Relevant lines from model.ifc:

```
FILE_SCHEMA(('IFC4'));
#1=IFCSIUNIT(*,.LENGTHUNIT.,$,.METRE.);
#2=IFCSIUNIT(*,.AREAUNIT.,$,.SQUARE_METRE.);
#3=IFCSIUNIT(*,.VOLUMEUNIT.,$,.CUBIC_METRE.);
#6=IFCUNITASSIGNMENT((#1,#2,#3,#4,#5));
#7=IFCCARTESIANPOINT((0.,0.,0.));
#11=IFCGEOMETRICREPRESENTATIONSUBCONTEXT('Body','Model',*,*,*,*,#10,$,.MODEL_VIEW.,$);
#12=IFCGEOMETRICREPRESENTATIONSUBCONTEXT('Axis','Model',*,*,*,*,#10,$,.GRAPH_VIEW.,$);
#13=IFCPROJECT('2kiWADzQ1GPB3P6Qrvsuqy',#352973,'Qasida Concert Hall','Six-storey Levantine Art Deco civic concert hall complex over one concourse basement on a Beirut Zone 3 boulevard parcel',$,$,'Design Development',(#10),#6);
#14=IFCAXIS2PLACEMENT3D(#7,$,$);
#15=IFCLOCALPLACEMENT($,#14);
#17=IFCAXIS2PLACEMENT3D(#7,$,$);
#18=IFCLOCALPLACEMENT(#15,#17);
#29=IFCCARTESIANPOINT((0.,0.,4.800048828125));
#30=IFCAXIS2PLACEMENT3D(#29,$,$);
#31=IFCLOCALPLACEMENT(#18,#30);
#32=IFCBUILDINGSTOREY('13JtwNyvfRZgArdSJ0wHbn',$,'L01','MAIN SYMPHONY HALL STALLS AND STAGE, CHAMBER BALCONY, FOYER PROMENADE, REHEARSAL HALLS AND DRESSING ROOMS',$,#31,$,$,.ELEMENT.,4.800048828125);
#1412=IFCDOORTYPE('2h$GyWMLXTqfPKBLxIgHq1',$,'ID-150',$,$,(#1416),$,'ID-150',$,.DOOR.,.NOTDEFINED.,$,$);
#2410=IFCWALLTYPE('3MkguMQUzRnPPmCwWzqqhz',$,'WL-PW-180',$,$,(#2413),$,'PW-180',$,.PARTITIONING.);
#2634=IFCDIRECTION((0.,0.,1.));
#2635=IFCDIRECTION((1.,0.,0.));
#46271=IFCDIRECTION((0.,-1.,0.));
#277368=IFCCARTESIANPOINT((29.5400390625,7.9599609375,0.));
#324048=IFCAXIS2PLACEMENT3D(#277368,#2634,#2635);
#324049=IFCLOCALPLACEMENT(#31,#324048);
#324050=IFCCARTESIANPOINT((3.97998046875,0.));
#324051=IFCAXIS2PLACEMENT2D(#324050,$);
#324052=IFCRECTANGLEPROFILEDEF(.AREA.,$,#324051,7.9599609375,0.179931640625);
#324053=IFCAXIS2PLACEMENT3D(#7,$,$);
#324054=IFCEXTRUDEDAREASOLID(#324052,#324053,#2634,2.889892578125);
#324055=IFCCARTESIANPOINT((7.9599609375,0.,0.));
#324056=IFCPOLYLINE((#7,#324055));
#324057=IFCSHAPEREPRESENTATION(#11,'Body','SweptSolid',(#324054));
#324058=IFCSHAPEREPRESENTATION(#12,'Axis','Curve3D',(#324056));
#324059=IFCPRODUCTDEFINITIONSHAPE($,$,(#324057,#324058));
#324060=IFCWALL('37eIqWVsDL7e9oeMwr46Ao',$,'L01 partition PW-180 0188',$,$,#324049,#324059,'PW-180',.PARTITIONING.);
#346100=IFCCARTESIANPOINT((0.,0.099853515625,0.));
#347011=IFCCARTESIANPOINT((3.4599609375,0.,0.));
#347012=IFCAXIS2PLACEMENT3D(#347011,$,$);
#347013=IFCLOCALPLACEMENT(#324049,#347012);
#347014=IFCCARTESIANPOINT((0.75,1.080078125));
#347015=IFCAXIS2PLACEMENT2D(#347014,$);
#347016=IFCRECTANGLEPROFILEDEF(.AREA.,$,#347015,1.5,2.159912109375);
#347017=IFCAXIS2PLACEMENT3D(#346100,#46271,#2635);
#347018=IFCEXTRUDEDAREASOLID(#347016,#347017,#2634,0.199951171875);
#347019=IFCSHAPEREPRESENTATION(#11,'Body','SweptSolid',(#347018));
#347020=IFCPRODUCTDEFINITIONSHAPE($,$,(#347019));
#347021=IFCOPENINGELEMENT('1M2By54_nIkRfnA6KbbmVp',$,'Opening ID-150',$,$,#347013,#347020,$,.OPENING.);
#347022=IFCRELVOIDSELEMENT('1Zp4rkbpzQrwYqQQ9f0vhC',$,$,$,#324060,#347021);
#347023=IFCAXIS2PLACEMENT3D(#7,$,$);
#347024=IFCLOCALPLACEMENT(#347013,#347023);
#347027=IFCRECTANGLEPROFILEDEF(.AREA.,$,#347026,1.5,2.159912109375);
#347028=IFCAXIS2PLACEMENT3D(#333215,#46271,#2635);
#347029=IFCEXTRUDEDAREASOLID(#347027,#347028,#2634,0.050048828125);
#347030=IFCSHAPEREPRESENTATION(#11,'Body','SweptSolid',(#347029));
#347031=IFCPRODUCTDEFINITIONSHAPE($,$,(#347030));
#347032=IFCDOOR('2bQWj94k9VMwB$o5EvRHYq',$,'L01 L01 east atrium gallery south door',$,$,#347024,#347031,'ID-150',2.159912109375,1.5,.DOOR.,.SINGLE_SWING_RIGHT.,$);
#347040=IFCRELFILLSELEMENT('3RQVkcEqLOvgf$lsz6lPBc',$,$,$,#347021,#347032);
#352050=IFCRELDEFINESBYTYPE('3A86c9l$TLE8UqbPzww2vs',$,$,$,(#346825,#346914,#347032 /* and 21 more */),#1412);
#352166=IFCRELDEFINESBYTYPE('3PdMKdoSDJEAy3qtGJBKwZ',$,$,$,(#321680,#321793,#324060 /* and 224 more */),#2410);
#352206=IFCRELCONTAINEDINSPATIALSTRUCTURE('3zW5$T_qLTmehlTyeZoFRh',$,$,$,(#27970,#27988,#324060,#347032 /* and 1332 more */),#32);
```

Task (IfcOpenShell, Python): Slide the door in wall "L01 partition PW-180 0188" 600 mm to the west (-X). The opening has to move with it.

```python
import ifcopenshell
import ifcopenshell.api.geometry
import ifcopenshell.util.placement

model = ifcopenshell.open("model.ifc")

door = model.by_guid("2bQWj94k9VMwB$o5EvRHYq")
opening = door.FillsVoids[0].RelatingOpeningElement
wall = opening.VoidsElements[0].RelatingBuildingElement

wall_matrix = ifcopenshell.util.placement.get_local_placement(wall.ObjectPlacement)
shift = wall_matrix[:3, 0] * -0.6
before = ifcopenshell.util.placement.get_local_placement(door.ObjectPlacement)[:3, 3].copy()

# The door is placed relative to its opening, so it follows when the opening moves.
matrix = ifcopenshell.util.placement.get_local_placement(opening.ObjectPlacement)
matrix[:3, 3] += shift
ifcopenshell.api.geometry.edit_object_placement(
    model, product=opening, matrix=matrix, is_si=False, should_transform_children=True
)

after = ifcopenshell.util.placement.get_local_placement(door.ObjectPlacement)[:3, 3]
print("door moved by", (after - before).round(3) + 0.0)

model.write("model-out.ifc")
```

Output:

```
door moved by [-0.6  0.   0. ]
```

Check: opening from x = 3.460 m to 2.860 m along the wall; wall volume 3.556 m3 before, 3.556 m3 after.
